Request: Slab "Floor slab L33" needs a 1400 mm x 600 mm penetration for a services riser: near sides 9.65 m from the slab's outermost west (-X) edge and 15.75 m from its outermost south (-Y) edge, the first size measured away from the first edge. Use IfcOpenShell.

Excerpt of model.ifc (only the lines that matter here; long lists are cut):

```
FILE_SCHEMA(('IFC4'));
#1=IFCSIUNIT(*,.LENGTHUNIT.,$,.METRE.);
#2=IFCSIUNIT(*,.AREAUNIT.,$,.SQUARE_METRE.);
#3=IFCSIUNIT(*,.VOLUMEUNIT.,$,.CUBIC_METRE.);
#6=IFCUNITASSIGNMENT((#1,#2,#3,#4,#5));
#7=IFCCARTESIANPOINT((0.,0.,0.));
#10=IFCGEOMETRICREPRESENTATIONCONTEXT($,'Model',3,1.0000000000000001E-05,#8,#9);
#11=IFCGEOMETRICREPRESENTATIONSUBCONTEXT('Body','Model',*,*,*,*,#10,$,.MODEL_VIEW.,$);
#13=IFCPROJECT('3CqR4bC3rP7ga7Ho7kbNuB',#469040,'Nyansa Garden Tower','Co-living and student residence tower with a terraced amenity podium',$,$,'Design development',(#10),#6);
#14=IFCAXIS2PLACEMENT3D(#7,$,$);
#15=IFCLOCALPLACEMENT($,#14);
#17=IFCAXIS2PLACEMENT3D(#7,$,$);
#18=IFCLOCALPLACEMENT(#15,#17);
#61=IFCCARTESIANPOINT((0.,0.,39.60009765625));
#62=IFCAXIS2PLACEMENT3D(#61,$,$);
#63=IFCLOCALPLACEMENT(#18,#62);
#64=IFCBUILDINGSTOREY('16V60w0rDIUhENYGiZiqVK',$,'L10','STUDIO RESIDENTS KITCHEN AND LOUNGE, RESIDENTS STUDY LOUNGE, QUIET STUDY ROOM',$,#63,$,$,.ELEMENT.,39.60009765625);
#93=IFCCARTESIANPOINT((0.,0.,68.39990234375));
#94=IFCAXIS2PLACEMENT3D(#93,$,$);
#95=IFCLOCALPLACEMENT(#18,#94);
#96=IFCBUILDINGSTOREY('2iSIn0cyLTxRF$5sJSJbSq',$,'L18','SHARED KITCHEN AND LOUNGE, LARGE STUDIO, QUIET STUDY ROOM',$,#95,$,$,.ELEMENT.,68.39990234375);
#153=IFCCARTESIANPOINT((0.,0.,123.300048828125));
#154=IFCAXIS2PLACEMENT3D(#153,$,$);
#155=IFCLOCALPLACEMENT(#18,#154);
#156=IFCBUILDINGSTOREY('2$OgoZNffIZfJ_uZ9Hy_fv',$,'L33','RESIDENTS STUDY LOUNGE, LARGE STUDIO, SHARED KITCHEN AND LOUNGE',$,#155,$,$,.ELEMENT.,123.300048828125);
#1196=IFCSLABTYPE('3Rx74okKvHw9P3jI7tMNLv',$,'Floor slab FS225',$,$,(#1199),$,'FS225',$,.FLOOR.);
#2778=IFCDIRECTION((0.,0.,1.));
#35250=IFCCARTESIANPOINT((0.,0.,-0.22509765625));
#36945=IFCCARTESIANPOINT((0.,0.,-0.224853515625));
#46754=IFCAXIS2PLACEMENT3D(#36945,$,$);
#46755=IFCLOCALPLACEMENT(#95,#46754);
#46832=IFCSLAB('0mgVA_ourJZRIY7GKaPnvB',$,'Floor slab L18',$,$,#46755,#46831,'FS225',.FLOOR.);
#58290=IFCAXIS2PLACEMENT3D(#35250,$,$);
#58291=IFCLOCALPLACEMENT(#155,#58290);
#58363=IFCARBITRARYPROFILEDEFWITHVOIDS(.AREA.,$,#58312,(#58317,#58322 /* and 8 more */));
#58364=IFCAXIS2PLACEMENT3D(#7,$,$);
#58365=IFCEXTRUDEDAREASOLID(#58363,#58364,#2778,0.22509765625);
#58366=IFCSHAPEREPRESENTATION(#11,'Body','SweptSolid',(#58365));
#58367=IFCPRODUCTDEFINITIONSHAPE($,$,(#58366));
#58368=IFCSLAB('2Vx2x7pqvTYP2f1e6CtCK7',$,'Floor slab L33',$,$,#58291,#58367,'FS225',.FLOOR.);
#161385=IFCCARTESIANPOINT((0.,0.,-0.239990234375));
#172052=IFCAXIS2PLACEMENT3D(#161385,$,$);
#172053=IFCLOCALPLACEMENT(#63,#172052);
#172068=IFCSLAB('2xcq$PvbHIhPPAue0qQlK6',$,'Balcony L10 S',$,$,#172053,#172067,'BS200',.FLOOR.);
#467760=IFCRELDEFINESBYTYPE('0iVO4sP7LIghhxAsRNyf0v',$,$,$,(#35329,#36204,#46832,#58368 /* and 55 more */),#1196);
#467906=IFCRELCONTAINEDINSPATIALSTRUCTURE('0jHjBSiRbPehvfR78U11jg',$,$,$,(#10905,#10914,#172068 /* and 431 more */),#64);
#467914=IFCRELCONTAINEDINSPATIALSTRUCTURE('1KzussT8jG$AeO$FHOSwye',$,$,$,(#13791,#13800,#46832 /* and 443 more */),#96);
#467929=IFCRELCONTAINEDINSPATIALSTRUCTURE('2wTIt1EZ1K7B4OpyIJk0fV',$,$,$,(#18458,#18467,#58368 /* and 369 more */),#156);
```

```python
import numpy as np
import ifcopenshell
import ifcopenshell.api.feature
import ifcopenshell.api.geometry
import ifcopenshell.api.root
import ifcopenshell.geom
import ifcopenshell.util.placement
import ifcopenshell.util.representation
import ifcopenshell.util.shape
import ifcopenshell.util.unit

model = ifcopenshell.open("model.ifc")
unit_scale = ifcopenshell.util.unit.calculate_unit_scale(model)
settings = ifcopenshell.geom.settings()


def volume(element):
    """Net volume in cubic metres, openings subtracted."""
    shape = ifcopenshell.geom.create_shape(settings, element)
    return ifcopenshell.util.shape.get_volume(shape.geometry)


slab = model.by_guid("2Vx2x7pqvTYP2f1e6CtCK7")
before = volume(slab)

# Extent in the slab's own axes, in metres. The edges named are its -X and -Y sides.
slab_shape = ifcopenshell.geom.create_shape(settings, slab)
vertices = ifcopenshell.util.shape.get_vertices(slab_shape.geometry)
x_min, y_min, bottom = vertices.min(axis=0)
top = vertices[:, 2].max()

opening = ifcopenshell.api.root.create_entity(model, ifc_class="IfcOpeningElement", name="Services riser opening", predefined_type="OPENING")
context = ifcopenshell.util.representation.get_context(model, "Model", "Body", "MODEL_VIEW")
width, depth = 1.4, 0.6
outline = [(0.0, 0.0), (width, 0.0), (width, depth), (0.0, depth), (0.0, 0.0)]
# Overshoot both faces by 50 mm so the cut is clean.
shape = ifcopenshell.api.geometry.add_slab_representation(
    model, context=context, depth=top - bottom + 0.1, polyline=outline
)
ifcopenshell.api.geometry.assign_representation(model, product=opening, representation=shape)

matrix = ifcopenshell.util.placement.get_local_placement(slab.ObjectPlacement)
matrix[:, 3] = matrix @ np.append(np.array([x_min + 9.65, y_min + 15.75, bottom - 0.05]) / unit_scale, 1.0)
ifcopenshell.api.geometry.edit_object_placement(model, product=opening, matrix=matrix, is_si=False)
ifcopenshell.api.feature.add_feature(model, feature=opening, element=slab)

after = volume(slab)

print(f"slab volume {before:.3f} -> {after:.3f} m3")

model.write("model-out.ifc")
```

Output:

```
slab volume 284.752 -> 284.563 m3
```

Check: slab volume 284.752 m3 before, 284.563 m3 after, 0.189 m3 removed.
